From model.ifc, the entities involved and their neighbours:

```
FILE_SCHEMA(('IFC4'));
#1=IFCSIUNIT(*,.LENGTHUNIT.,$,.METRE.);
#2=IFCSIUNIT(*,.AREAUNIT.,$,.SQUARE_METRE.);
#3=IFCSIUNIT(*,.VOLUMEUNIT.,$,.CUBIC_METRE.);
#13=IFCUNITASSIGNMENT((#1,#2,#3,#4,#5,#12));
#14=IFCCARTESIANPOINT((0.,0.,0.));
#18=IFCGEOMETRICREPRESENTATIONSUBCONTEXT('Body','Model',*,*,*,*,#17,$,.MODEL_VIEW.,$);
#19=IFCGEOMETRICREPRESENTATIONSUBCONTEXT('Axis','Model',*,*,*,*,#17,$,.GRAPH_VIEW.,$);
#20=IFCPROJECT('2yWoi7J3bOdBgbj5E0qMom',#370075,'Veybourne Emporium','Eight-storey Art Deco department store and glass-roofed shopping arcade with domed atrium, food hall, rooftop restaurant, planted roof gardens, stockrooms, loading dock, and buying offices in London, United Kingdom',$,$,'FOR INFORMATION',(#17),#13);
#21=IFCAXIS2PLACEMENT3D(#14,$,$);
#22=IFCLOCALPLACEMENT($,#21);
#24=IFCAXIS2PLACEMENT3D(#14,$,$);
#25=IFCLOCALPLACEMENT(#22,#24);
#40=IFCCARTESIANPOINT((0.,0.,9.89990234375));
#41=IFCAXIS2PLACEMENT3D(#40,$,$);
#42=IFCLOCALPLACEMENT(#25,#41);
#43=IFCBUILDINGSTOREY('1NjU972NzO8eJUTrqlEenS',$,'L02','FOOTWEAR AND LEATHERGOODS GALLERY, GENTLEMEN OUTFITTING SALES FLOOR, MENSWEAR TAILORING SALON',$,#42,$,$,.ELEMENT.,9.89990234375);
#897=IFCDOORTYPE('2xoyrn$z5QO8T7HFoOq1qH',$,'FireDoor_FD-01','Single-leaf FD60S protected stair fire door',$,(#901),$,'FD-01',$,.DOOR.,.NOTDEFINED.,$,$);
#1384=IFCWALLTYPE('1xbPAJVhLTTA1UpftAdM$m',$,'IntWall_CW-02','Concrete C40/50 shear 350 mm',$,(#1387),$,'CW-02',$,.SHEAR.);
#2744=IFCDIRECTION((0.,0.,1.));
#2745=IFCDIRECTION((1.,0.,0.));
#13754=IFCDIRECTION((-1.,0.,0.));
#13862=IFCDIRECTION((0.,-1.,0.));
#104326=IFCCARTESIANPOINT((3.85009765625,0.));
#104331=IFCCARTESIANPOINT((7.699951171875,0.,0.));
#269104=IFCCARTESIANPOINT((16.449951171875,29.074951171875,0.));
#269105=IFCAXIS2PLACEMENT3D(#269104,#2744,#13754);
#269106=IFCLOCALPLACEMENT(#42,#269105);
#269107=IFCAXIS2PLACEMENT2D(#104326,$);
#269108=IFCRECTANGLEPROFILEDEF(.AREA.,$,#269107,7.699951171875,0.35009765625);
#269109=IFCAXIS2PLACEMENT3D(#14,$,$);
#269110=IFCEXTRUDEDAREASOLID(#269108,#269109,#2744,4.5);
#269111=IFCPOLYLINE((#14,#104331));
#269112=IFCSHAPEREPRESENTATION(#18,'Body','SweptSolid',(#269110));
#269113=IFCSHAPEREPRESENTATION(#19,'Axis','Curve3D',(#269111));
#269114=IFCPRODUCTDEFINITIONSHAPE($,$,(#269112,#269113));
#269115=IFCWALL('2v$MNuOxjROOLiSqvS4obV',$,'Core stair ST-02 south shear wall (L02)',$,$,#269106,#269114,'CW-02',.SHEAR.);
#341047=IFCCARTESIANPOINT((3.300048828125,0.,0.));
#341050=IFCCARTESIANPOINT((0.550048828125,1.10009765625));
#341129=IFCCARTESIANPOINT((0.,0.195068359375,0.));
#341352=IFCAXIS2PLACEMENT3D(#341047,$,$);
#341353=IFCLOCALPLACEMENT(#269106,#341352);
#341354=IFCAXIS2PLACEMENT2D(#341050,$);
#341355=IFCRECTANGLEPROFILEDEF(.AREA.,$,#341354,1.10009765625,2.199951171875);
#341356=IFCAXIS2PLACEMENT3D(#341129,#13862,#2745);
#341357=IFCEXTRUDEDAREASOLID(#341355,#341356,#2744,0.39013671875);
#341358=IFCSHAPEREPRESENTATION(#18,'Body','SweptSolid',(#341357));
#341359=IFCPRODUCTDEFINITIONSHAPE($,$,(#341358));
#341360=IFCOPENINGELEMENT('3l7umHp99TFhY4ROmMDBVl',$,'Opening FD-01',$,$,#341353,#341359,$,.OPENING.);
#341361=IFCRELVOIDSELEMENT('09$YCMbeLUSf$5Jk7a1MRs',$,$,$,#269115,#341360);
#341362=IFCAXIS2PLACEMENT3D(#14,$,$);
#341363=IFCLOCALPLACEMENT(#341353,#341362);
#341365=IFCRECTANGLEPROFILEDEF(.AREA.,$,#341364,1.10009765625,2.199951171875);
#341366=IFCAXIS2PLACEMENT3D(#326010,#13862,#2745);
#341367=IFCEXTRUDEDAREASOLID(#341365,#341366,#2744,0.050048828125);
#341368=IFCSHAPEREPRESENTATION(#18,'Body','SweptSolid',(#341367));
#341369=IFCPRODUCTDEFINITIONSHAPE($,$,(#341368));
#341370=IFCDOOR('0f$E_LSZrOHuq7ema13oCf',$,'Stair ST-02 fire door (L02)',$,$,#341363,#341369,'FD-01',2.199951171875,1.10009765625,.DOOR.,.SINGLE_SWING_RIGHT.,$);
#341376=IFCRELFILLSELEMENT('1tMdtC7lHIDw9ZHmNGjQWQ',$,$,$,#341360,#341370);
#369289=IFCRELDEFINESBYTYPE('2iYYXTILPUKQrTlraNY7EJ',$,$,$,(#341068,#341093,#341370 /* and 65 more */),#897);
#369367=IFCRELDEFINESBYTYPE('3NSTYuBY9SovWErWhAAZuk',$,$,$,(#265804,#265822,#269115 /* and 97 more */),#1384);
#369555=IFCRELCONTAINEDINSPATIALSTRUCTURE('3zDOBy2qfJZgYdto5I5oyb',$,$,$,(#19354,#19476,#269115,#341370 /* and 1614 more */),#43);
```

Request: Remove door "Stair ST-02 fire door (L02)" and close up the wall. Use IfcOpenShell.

```python
import ifcopenshell
import ifcopenshell.api.feature
import ifcopenshell.api.root
import ifcopenshell.geom
import ifcopenshell.util.shape

model = ifcopenshell.open("model.ifc")
settings = ifcopenshell.geom.settings()


def volume(element):
    """Net volume in cubic metres, openings subtracted."""
    shape = ifcopenshell.geom.create_shape(settings, element)
    return ifcopenshell.util.shape.get_volume(shape.geometry)


door = model.by_guid("0f$E_LSZrOHuq7ema13oCf")
opening = door.FillsVoids[0].RelatingOpeningElement
wall = opening.VoidsElements[0].RelatingBuildingElement
before = volume(wall)

ifcopenshell.api.root.remove_product(model, product=door)
ifcopenshell.api.feature.remove_feature(model, feature=opening)

after = volume(wall)

print(f"wall volume {before:.3f} -> {after:.3f} m3")

model.write("model-out.ifc")
```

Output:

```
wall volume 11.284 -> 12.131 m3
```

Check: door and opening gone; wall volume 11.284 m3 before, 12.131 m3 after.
